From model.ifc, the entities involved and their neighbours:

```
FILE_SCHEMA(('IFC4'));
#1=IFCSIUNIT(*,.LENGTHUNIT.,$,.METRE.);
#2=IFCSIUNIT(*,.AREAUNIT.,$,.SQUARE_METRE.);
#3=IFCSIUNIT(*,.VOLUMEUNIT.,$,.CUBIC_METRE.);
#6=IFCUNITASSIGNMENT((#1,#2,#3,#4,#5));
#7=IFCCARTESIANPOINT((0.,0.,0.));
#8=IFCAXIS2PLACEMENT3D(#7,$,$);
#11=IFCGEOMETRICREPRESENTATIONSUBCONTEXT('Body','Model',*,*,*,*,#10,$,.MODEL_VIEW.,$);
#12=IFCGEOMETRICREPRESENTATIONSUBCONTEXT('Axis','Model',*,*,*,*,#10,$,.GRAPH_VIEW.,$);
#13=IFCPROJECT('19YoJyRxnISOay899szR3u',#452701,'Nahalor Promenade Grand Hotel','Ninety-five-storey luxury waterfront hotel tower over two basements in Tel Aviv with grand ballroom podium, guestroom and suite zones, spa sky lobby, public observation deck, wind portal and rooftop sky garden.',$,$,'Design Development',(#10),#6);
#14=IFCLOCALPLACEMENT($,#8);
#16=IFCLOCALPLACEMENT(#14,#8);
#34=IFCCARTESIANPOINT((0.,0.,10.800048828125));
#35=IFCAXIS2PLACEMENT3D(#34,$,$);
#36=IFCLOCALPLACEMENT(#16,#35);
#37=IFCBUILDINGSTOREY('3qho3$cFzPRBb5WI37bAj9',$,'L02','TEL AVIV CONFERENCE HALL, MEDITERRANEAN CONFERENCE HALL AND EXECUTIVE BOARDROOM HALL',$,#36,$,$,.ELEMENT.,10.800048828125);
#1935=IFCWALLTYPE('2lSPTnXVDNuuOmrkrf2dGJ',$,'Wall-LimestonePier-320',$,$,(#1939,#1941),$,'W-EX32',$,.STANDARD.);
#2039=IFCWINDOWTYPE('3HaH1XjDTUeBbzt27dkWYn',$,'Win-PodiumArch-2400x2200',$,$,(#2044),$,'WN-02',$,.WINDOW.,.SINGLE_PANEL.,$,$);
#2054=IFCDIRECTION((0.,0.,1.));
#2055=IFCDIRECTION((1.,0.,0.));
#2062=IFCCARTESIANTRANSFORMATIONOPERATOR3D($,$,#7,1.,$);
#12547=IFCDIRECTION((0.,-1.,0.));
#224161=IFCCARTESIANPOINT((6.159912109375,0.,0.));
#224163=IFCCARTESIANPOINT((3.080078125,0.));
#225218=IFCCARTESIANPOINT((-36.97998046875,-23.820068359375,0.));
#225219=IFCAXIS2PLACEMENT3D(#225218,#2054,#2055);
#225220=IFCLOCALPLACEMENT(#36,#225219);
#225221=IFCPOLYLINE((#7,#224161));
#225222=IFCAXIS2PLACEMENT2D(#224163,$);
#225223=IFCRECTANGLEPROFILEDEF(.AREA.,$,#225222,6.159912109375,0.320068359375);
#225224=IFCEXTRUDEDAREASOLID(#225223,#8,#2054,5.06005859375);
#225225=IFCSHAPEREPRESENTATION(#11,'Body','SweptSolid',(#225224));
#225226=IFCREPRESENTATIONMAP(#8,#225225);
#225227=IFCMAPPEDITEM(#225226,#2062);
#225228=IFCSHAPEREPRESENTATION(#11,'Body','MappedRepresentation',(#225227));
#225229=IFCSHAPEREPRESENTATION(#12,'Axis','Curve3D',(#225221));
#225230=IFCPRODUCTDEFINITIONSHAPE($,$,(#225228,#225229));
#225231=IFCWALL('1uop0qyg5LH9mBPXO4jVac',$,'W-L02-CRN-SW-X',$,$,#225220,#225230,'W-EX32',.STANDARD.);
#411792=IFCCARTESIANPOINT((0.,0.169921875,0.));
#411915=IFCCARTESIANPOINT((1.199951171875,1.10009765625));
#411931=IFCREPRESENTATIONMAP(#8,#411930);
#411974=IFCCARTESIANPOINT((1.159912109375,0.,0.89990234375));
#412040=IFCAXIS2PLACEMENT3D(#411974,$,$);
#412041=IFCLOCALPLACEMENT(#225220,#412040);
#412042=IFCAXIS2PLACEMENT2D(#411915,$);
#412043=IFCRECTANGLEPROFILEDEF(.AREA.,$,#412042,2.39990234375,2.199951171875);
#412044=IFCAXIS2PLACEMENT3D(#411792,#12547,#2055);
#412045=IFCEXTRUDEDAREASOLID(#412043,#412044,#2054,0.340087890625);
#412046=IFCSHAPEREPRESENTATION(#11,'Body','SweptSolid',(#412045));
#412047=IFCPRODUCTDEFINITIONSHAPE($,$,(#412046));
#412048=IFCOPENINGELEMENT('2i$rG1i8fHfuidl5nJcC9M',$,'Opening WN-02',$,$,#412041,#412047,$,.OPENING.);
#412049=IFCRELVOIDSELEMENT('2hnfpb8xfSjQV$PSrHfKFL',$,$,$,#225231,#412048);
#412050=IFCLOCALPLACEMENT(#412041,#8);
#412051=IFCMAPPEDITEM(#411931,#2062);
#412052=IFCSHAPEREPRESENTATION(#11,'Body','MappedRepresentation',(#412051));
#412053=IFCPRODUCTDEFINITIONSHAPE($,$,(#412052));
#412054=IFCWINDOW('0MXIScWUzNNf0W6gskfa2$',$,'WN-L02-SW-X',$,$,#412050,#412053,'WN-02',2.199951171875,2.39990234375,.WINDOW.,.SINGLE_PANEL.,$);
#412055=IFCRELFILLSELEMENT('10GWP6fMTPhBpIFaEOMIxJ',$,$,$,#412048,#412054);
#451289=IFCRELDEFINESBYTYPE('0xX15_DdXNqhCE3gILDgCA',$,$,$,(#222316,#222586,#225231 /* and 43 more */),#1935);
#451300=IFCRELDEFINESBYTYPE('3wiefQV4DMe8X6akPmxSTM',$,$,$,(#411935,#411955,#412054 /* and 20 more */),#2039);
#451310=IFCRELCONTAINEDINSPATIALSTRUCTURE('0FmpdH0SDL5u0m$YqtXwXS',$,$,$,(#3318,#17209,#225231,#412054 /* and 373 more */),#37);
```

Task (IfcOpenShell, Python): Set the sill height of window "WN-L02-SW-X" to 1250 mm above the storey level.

```python
import numpy as np
import ifcopenshell
import ifcopenshell.api.geometry
import ifcopenshell.geom
import ifcopenshell.util.element
import ifcopenshell.util.placement
import ifcopenshell.util.shape
import ifcopenshell.util.unit

model = ifcopenshell.open("model.ifc")
unit_scale = ifcopenshell.util.unit.calculate_unit_scale(model)

window = model.by_id(412054)
opening = window.FillsVoids[0].RelatingOpeningElement
storey = ifcopenshell.util.element.get_container(window, ifc_class="IfcBuildingStorey")
level = ifcopenshell.util.placement.get_local_placement(storey.ObjectPlacement)[2, 3]

# The opening's origin need not be at the sill, so measure its lowest point.
shape = ifcopenshell.geom.create_shape(ifcopenshell.geom.settings(), opening)
bottom = ifcopenshell.util.shape.get_shape_bottom_elevation(shape, shape.geometry) / unit_scale
dz = level + 1.25 - bottom

shift = np.array([0.0, 0.0, dz])
# The window is placed relative to its opening, so it follows when the opening moves.
matrix = ifcopenshell.util.placement.get_local_placement(opening.ObjectPlacement)
matrix[:3, 3] += shift
ifcopenshell.api.geometry.edit_object_placement(
    model, product=opening, matrix=matrix, is_si=False, should_transform_children=True
)

print(f"moved by {dz * unit_scale:+.3f} m")

model.write("model_updated.ifc")
```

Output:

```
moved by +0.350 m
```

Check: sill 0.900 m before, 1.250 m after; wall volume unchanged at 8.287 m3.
